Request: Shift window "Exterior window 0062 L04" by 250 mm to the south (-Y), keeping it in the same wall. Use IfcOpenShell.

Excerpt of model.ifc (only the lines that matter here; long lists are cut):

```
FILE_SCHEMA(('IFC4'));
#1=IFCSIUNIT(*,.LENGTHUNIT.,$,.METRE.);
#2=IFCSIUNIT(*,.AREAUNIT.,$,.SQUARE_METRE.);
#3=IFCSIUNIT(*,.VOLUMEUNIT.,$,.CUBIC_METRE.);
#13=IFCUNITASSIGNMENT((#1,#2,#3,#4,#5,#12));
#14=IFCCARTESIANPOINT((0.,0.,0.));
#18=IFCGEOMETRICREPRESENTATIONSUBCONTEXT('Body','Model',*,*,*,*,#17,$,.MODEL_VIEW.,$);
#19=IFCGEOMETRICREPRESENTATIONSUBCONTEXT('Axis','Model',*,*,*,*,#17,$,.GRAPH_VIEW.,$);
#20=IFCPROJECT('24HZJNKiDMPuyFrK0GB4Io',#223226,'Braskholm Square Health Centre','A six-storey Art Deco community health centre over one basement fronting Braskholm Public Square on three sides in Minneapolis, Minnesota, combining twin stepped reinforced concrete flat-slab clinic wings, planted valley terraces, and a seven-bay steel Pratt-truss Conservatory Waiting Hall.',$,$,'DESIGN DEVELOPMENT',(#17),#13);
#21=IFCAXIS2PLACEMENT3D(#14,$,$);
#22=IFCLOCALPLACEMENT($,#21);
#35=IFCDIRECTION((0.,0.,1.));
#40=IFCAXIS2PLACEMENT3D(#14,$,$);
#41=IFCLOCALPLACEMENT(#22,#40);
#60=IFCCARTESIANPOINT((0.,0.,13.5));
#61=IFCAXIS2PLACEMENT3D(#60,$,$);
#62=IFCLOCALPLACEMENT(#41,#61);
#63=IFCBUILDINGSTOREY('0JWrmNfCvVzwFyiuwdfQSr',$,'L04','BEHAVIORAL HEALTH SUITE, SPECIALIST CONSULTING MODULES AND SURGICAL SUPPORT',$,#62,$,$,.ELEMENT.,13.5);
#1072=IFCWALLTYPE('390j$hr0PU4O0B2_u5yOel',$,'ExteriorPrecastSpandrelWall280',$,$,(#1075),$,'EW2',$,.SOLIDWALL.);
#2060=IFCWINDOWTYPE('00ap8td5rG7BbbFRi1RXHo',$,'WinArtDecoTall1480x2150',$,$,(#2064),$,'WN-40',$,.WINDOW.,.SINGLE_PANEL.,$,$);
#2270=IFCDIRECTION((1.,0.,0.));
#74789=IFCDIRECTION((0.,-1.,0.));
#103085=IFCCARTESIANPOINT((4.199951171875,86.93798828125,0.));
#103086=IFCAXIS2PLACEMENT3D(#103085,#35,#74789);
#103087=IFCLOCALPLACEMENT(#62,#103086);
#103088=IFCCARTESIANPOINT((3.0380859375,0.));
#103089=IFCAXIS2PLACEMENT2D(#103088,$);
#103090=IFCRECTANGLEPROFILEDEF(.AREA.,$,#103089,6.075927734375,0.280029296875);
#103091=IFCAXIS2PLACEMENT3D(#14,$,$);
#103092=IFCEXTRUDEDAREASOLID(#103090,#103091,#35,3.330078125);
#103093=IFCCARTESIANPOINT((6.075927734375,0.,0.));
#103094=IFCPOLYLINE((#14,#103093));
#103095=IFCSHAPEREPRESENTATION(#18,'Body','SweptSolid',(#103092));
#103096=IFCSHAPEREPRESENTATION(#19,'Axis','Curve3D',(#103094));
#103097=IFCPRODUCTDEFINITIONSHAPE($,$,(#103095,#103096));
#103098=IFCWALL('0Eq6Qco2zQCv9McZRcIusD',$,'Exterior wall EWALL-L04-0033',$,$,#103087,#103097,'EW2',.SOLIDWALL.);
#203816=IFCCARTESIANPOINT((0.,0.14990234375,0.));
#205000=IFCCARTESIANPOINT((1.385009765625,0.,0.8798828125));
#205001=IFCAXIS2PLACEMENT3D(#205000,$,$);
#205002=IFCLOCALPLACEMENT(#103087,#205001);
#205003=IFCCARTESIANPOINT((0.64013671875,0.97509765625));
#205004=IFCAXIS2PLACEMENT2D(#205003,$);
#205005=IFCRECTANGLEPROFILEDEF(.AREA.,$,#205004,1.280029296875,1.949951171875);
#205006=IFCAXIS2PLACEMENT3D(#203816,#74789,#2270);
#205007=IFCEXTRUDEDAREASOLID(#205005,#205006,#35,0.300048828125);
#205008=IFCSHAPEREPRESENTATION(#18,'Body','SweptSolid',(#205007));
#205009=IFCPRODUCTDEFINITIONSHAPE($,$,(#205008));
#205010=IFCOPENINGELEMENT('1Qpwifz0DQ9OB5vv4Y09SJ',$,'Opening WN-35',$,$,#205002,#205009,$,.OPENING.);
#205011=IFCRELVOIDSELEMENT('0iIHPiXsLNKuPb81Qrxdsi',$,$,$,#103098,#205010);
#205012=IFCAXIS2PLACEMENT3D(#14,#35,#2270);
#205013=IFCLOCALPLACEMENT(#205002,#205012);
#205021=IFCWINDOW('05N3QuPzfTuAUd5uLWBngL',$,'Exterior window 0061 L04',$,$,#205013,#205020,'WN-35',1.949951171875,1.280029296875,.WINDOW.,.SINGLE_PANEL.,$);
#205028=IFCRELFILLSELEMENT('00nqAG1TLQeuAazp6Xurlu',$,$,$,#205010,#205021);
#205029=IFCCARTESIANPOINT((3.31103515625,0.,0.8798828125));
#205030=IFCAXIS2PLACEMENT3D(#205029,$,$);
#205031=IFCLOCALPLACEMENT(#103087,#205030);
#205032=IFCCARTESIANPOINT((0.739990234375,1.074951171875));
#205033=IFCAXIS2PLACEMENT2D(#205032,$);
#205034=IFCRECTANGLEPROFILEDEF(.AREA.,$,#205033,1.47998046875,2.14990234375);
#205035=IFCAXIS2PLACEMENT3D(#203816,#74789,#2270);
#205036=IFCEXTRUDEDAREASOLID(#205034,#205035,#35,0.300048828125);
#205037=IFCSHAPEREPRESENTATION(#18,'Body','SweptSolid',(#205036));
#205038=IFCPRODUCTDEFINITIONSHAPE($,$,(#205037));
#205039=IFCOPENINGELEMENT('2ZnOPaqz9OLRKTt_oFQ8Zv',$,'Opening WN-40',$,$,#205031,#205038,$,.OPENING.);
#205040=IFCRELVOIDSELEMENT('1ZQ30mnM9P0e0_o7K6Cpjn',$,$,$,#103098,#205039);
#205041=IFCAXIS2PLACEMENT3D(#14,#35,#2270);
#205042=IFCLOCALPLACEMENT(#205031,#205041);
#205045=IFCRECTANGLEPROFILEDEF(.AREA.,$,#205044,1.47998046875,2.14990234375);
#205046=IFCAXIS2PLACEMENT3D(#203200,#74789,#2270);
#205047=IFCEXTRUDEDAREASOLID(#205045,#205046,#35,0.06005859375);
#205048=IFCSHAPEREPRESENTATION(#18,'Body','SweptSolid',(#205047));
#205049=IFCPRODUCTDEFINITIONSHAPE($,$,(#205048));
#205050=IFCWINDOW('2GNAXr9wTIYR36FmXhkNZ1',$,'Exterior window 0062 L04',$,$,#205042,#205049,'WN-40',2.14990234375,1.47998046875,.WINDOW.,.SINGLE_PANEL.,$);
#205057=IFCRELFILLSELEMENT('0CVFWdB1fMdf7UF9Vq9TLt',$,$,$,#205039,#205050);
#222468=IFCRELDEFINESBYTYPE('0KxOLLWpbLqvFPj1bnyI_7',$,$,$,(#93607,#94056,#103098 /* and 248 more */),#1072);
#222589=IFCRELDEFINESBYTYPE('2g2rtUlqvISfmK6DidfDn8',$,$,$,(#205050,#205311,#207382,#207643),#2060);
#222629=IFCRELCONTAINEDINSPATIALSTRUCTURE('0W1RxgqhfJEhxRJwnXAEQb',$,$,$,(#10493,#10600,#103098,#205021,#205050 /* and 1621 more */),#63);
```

```python
import ifcopenshell
import ifcopenshell.api.geometry
import ifcopenshell.util.placement

model = ifcopenshell.open("model.ifc")

window = model.by_guid("2GNAXr9wTIYR36FmXhkNZ1")
opening = window.FillsVoids[0].RelatingOpeningElement
wall = opening.VoidsElements[0].RelatingBuildingElement

wall_matrix = ifcopenshell.util.placement.get_local_placement(wall.ObjectPlacement)
shift = wall_matrix[:3, 0] * 0.25
before = ifcopenshell.util.placement.get_local_placement(window.ObjectPlacement)[:3, 3].copy()

# The window is placed relative to its opening, so it follows when the opening moves.
matrix = ifcopenshell.util.placement.get_local_placement(opening.ObjectPlacement)
matrix[:3, 3] += shift
ifcopenshell.api.geometry.edit_object_placement(
    model, product=opening, matrix=matrix, is_si=False, should_transform_children=True
)

after = ifcopenshell.util.placement.get_local_placement(window.ObjectPlacement)[:3, 3]
print("window moved by", (after - before).round(3) + 0.0)

model.write("model_updated.ifc")
```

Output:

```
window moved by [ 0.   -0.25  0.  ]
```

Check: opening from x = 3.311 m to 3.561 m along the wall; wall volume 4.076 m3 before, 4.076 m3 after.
